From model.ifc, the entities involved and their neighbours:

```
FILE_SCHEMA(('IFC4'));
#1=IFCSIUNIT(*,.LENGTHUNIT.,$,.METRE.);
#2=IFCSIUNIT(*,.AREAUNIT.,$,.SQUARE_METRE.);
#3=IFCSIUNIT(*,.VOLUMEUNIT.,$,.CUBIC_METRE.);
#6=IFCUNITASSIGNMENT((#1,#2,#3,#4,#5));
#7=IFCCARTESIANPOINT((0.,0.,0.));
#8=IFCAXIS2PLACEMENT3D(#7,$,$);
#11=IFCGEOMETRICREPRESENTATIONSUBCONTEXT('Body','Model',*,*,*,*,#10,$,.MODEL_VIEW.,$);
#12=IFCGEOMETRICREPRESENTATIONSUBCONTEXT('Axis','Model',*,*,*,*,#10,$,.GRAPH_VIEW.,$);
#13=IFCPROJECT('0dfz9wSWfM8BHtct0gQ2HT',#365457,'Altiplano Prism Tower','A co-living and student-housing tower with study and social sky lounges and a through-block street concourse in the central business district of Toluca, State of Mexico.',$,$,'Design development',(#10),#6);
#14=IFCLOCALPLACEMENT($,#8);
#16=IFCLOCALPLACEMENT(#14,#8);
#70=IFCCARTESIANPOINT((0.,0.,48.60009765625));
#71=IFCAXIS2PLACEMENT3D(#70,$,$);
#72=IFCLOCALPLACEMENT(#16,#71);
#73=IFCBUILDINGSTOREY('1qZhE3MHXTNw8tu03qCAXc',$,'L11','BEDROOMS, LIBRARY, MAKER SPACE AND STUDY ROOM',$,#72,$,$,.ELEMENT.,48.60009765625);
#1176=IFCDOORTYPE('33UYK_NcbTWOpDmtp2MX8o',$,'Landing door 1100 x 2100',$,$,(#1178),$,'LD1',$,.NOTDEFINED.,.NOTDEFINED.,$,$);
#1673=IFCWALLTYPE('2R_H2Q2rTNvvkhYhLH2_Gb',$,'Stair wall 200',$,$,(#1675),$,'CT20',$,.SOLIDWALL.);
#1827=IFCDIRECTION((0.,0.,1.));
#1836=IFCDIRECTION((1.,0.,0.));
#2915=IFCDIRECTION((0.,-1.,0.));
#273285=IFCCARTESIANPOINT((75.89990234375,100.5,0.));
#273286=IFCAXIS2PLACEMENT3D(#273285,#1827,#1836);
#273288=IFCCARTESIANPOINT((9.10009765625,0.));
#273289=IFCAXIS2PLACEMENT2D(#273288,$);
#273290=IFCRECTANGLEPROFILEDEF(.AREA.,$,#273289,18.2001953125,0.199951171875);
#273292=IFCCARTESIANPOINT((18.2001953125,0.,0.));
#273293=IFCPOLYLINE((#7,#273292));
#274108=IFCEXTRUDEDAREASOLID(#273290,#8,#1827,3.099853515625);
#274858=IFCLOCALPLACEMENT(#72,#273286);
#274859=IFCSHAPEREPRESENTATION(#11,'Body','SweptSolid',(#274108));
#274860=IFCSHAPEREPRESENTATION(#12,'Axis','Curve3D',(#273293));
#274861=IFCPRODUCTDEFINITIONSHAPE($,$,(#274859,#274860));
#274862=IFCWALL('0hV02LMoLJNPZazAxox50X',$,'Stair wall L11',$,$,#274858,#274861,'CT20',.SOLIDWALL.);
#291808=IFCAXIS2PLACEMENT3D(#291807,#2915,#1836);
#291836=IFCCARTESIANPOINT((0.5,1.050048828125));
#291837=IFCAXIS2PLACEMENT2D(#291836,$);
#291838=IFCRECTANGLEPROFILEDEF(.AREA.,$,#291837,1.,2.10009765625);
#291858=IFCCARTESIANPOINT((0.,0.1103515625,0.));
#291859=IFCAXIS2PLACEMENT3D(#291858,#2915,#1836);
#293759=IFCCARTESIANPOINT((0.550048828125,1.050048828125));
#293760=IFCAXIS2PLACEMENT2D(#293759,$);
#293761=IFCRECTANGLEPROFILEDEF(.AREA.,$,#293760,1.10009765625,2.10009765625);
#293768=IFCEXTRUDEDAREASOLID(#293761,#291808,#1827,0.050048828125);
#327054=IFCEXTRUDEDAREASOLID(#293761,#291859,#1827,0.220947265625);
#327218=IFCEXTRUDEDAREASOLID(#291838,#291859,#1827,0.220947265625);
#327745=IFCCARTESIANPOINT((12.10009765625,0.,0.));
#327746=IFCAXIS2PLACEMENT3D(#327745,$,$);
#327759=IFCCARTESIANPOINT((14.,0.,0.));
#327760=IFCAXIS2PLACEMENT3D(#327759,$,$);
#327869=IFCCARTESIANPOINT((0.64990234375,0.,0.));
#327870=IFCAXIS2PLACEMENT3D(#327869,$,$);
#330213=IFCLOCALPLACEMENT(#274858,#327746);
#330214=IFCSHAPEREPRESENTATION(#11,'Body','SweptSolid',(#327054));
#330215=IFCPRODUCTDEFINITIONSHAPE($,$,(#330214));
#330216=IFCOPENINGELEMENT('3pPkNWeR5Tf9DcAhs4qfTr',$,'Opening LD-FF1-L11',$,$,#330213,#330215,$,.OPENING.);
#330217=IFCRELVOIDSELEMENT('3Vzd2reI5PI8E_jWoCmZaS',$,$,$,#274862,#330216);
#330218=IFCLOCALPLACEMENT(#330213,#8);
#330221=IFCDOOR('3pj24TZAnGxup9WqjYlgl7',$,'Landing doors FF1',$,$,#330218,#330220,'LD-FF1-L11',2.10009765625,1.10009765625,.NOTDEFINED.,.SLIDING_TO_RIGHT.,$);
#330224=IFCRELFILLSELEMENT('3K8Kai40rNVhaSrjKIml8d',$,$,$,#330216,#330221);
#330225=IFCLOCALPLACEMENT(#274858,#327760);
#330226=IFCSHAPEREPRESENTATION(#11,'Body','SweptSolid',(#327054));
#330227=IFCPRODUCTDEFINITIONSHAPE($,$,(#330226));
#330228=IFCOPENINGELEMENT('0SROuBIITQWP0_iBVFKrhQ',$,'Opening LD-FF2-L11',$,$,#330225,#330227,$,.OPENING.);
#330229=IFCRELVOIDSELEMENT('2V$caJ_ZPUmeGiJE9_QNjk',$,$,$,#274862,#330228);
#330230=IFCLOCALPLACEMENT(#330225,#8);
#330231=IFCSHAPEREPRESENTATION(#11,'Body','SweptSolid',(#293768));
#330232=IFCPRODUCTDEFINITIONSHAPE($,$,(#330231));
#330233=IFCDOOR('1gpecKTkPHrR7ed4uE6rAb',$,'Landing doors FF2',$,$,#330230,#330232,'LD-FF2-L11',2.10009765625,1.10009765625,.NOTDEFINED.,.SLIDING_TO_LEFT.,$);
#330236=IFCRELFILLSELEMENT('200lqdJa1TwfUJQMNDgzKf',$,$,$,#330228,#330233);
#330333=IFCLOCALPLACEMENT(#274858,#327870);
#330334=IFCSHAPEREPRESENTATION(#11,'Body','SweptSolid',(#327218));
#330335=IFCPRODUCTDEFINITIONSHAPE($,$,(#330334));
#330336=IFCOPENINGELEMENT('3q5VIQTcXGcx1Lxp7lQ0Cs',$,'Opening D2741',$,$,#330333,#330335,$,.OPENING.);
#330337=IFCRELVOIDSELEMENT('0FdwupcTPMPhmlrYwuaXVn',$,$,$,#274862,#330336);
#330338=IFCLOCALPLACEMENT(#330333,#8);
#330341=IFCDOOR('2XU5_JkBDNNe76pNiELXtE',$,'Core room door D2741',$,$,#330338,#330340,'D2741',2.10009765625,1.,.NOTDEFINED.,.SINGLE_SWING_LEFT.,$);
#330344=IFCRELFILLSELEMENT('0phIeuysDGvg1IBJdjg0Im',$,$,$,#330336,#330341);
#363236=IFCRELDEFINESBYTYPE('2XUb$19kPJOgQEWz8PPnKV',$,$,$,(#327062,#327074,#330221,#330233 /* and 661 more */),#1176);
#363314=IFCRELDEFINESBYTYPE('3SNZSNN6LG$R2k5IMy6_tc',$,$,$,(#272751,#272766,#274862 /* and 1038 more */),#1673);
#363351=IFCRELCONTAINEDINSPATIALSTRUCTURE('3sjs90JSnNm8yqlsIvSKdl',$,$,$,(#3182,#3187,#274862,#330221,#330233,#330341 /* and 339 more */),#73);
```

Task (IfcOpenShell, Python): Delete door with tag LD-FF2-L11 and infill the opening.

```python
import ifcopenshell
import ifcopenshell.api.feature
import ifcopenshell.api.root
import ifcopenshell.geom
import ifcopenshell.util.shape

model = ifcopenshell.open("model.ifc")
settings = ifcopenshell.geom.settings()


def volume(element):
    """Net volume in cubic metres, openings subtracted."""
    shape = ifcopenshell.geom.create_shape(settings, element)
    return ifcopenshell.util.shape.get_volume(shape.geometry)


door = model.by_guid("1gpecKTkPHrR7ed4uE6rAb")
opening = door.FillsVoids[0].RelatingOpeningElement
wall = opening.VoidsElements[0].RelatingBuildingElement
before = volume(wall)

ifcopenshell.api.root.remove_product(model, product=door)
ifcopenshell.api.feature.remove_feature(model, feature=opening)

after = volume(wall)

print(f"wall volume {before:.3f} -> {after:.3f} m3")

model.write("model-out.ifc")
```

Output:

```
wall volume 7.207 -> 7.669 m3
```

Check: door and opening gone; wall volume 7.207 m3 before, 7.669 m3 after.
